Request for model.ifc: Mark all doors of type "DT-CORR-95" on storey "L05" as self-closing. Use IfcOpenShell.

First a look at what the model holds.

```python
import ifcopenshell
import ifcopenshell.util.element

model = ifcopenshell.open("model.ifc")
print(model.schema)
storey = next(s for s in model.by_type("IfcBuildingStorey") if s.Name == "L05")
doors = [e for e in ifcopenshell.util.element.get_decomposition(storey) if e.is_a("IfcDoor")]
seen = {}
for e in doors:
    element_type = ifcopenshell.util.element.get_type(e)
    key = (element_type.Name if element_type != e and element_type else None, ifcopenshell.util.element.get_pset(e, "Pset_DoorCommon", "SelfClosing"))
    seen[key] = seen.get(key, 0) + 1
for (name, value), count in sorted(seen.items(), key=str):
    print(count, "x", name, "|", value)
```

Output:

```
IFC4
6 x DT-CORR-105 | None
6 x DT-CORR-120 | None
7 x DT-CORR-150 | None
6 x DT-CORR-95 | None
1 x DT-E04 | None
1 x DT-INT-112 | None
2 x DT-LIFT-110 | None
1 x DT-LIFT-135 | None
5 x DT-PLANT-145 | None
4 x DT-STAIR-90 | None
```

```python
import ifcopenshell
import ifcopenshell.api.pset
import ifcopenshell.util.element

model = ifcopenshell.open("model.ifc")

storey = next(s for s in model.by_type("IfcBuildingStorey") if s.Name == "L05")
doors = [e for e in ifcopenshell.util.element.get_decomposition(storey) if e.is_a("IfcDoor")]

count = 0
for e in doors:
    element_type = ifcopenshell.util.element.get_type(e)
    if element_type in (None, e) or element_type.Name != "DT-CORR-95":
        continue
    # add_pset returns the element's existing set when there is one.
    pset = ifcopenshell.api.pset.add_pset(model, product=e, name="Pset_DoorCommon")
    ifcopenshell.api.pset.edit_pset(model, pset=pset, properties={"SelfClosing": True})
    count += 1

print(count, "doors updated")

model.write("model_edited.ifc")
```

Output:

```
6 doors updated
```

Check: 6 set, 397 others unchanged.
